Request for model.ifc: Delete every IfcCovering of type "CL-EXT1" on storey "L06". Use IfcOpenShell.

First a look at what the model holds.

```python
import ifcopenshell
import ifcopenshell.util.element

model = ifcopenshell.open("model.ifc")
print(model.schema)
storey = next(s for s in model.by_type("IfcBuildingStorey") if s.Name == "L06")
coverings = [e for e in ifcopenshell.util.element.get_decomposition(storey) if e.is_a("IfcCovering")]
seen = {}
for e in coverings:
    element_type = ifcopenshell.util.element.get_type(e)
    name = element_type.Name if element_type not in (None, e) else None
    seen[name] = seen.get(name, 0) + 1
for name, count in sorted(seen.items(), key=str):
    print(count, "x", name)
```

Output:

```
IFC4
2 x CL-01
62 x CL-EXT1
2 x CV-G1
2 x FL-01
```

```python
import ifcopenshell
import ifcopenshell.api.root
import ifcopenshell.util.element

model = ifcopenshell.open("model.ifc")

storey = next(s for s in model.by_type("IfcBuildingStorey") if s.Name == "L06")
coverings = [e for e in ifcopenshell.util.element.get_decomposition(storey) if e.is_a("IfcCovering")]
targets = [e for e in coverings if (t := ifcopenshell.util.element.get_type(e)) not in (None, e) and t.Name == "CL-EXT1"]

for e in targets:
    ifcopenshell.api.root.remove_product(model, product=e)
print(len(targets), "removed")

model.write("model_rev.ifc")
```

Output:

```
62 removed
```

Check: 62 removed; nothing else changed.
